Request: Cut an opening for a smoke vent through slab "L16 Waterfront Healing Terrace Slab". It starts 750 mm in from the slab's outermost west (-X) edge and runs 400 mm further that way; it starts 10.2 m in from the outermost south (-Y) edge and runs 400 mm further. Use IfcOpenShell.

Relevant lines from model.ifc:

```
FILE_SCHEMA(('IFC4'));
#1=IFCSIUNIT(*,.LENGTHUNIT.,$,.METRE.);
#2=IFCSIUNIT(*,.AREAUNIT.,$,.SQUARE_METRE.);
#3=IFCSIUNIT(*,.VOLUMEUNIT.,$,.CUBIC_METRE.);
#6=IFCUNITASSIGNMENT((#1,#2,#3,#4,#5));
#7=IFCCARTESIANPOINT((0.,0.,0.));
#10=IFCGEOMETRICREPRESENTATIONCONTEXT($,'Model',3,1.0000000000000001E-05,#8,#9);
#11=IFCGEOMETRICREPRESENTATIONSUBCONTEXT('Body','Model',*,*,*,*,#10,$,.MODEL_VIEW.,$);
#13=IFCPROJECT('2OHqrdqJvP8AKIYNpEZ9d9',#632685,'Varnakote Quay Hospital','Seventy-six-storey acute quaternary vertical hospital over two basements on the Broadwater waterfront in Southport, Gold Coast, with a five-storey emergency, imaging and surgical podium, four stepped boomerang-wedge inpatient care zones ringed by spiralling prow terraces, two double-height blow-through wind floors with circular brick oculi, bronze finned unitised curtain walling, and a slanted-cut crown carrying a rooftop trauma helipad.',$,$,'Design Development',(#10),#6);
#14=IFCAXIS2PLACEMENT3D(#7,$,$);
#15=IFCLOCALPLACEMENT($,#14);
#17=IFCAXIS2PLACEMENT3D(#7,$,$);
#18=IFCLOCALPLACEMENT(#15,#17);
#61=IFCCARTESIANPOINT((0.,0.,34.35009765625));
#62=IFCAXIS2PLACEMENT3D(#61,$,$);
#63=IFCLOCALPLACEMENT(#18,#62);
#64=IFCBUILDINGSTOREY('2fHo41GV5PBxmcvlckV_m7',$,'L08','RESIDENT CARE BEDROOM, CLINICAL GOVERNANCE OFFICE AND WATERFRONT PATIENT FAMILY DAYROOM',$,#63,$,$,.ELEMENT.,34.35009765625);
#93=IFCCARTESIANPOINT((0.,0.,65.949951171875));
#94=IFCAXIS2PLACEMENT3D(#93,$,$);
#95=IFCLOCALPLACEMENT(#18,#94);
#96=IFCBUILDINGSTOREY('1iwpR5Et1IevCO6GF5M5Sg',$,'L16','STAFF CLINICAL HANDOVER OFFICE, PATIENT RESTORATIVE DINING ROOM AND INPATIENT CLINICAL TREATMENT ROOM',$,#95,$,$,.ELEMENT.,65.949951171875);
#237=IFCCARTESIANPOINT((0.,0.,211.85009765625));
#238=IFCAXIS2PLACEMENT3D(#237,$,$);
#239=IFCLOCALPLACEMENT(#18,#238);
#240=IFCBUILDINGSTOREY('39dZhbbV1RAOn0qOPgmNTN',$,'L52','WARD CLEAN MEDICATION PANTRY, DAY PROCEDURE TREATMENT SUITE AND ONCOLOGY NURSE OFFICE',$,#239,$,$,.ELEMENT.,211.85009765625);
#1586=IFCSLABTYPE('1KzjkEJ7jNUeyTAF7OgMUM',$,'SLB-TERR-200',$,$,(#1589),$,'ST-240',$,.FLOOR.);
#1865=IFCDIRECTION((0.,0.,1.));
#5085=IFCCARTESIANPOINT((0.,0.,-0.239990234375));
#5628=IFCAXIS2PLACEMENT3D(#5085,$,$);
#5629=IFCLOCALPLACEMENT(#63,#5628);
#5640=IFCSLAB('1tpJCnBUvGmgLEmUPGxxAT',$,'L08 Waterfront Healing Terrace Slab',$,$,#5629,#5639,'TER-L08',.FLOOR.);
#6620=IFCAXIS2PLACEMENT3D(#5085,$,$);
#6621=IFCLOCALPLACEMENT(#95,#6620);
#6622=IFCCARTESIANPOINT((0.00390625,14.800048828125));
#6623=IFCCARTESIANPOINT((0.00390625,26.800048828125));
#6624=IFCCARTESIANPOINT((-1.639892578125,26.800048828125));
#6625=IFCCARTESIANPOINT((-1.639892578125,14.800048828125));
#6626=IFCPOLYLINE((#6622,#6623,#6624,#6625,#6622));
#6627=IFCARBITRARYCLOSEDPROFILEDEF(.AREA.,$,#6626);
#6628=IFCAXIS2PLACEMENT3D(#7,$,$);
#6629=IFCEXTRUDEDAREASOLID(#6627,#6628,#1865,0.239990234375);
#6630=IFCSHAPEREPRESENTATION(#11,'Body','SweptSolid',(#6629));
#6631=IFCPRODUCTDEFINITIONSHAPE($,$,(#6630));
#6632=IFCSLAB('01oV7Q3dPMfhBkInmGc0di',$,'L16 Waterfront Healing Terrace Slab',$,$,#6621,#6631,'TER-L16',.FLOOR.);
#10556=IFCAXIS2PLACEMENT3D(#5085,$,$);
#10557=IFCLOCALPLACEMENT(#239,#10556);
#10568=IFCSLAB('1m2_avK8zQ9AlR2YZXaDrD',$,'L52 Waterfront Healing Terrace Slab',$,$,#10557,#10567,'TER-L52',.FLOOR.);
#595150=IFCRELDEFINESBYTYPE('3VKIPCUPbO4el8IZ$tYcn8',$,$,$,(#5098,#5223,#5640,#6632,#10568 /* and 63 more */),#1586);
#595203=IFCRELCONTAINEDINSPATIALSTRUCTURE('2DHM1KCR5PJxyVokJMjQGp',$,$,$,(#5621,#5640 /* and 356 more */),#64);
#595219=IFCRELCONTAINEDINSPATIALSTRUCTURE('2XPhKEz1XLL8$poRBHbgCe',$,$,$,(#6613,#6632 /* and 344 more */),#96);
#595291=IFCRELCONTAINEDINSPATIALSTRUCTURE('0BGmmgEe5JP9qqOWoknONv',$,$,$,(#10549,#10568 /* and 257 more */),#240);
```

```python
import numpy as np
import ifcopenshell
import ifcopenshell.api.feature
import ifcopenshell.api.geometry
import ifcopenshell.api.root
import ifcopenshell.geom
import ifcopenshell.util.placement
import ifcopenshell.util.representation
import ifcopenshell.util.shape
import ifcopenshell.util.unit

model = ifcopenshell.open("model.ifc")
unit_scale = ifcopenshell.util.unit.calculate_unit_scale(model)
settings = ifcopenshell.geom.settings()


def volume(element):
    """Net volume in cubic metres, openings subtracted."""
    shape = ifcopenshell.geom.create_shape(settings, element)
    return ifcopenshell.util.shape.get_volume(shape.geometry)


slab = model.by_guid("01oV7Q3dPMfhBkInmGc0di")
before = volume(slab)

# Extent in the slab's own axes, in metres. The edges named are its -X and -Y sides.
slab_shape = ifcopenshell.geom.create_shape(settings, slab)
vertices = ifcopenshell.util.shape.get_vertices(slab_shape.geometry)
x_min, y_min, bottom = vertices.min(axis=0)
top = vertices[:, 2].max()

opening = ifcopenshell.api.root.create_entity(model, ifc_class="IfcOpeningElement", name="Smoke vent opening", predefined_type="OPENING")
context = ifcopenshell.util.representation.get_context(model, "Model", "Body", "MODEL_VIEW")
width, depth = 0.4, 0.4
outline = [(0.0, 0.0), (width, 0.0), (width, depth), (0.0, depth), (0.0, 0.0)]
# Overshoot both faces by 50 mm so the cut is clean.
shape = ifcopenshell.api.geometry.add_slab_representation(
    model, context=context, depth=top - bottom + 0.1, polyline=outline
)
ifcopenshell.api.geometry.assign_representation(model, product=opening, representation=shape)

matrix = ifcopenshell.util.placement.get_local_placement(slab.ObjectPlacement)
matrix[:, 3] = matrix @ np.append(np.array([x_min + 0.75, y_min + 10.2, bottom - 0.05]) / unit_scale, 1.0)
ifcopenshell.api.geometry.edit_object_placement(model, product=opening, matrix=matrix, is_si=False)
ifcopenshell.api.feature.add_feature(model, feature=opening, element=slab)

after = volume(slab)

print(f"slab volume {before:.3f} -> {after:.3f} m3")

model.write("model_updated.ifc")
```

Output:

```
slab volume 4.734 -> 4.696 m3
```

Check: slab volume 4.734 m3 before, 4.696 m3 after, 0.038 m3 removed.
